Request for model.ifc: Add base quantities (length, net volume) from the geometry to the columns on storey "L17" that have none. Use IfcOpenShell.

First a look at what the model holds.

```python
import ifcopenshell
import ifcopenshell.util.element
import ifcopenshell.util.unit

model = ifcopenshell.open("model.ifc")
print(model.schema)
for unit_type in ("LENGTHUNIT", "AREAUNIT", "VOLUMEUNIT"):
    print(unit_type, ifcopenshell.util.unit.calculate_unit_scale(model, unit_type))
storey = next(s for s in model.by_type("IfcBuildingStorey") if s.Name == "L17")
columns = [e for e in ifcopenshell.util.element.get_decomposition(storey) if e.is_a("IfcColumn")]
for e in sorted(columns, key=lambda e: e.id()):
    print(e.id(), e.is_a(), e.Name, list(ifcopenshell.util.element.get_psets(e, qtos_only=True)), sep=" | ")
```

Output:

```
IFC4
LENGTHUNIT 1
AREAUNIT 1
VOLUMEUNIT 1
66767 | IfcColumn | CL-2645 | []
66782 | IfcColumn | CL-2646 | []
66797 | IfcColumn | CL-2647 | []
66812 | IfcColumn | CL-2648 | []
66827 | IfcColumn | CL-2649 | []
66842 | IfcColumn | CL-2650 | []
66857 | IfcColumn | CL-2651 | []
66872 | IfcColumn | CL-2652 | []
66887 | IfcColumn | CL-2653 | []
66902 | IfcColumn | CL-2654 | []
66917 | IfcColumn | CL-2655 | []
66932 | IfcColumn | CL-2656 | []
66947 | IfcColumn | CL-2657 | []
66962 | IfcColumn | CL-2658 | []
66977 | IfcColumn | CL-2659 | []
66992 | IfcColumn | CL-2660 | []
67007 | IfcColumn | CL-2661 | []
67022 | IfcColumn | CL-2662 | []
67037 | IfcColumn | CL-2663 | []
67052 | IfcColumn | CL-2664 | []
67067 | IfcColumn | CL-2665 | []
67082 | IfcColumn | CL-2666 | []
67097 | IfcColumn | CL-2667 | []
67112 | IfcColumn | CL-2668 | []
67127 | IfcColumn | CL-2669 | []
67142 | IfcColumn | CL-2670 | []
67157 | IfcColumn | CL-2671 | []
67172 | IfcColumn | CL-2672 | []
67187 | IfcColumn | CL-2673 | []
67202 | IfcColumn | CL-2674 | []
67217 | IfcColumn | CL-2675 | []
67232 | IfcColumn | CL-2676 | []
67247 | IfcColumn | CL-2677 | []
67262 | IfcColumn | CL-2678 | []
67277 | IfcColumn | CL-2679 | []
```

```python
import ifcopenshell
import ifcopenshell.api.pset
import ifcopenshell.geom
import ifcopenshell.util.element
import ifcopenshell.util.shape
import ifcopenshell.util.unit

model = ifcopenshell.open("model.ifc")
unit_scale = ifcopenshell.util.unit.calculate_unit_scale(model)
volume_scale = ifcopenshell.util.unit.calculate_unit_scale(model, "VOLUMEUNIT")
settings = ifcopenshell.geom.settings()

storey = next(s for s in model.by_type("IfcBuildingStorey") if s.Name == "L17")
columns = [e for e in ifcopenshell.util.element.get_decomposition(storey) if e.is_a("IfcColumn")]

for e in sorted(columns, key=lambda e: e.id()):
    if ifcopenshell.util.element.get_psets(e, qtos_only=True, should_inherit=False):
        continue
    # Geometry comes back in metres, in the element's own axes.
    shape = ifcopenshell.geom.create_shape(settings, e)
    values = {
        "Length": ifcopenshell.util.shape.get_z(shape.geometry) / unit_scale,
        "NetVolume": ifcopenshell.util.shape.get_volume(shape.geometry) / volume_scale,
    }
    qto = ifcopenshell.api.pset.add_qto(model, product=e, name="Qto_ColumnBaseQuantities")
    ifcopenshell.api.pset.edit_qto(model, qto=qto, properties=values)
    print(e.id(), {k: round(v, 3) for k, v in values.items()})

model.write("model_updated.ifc")
```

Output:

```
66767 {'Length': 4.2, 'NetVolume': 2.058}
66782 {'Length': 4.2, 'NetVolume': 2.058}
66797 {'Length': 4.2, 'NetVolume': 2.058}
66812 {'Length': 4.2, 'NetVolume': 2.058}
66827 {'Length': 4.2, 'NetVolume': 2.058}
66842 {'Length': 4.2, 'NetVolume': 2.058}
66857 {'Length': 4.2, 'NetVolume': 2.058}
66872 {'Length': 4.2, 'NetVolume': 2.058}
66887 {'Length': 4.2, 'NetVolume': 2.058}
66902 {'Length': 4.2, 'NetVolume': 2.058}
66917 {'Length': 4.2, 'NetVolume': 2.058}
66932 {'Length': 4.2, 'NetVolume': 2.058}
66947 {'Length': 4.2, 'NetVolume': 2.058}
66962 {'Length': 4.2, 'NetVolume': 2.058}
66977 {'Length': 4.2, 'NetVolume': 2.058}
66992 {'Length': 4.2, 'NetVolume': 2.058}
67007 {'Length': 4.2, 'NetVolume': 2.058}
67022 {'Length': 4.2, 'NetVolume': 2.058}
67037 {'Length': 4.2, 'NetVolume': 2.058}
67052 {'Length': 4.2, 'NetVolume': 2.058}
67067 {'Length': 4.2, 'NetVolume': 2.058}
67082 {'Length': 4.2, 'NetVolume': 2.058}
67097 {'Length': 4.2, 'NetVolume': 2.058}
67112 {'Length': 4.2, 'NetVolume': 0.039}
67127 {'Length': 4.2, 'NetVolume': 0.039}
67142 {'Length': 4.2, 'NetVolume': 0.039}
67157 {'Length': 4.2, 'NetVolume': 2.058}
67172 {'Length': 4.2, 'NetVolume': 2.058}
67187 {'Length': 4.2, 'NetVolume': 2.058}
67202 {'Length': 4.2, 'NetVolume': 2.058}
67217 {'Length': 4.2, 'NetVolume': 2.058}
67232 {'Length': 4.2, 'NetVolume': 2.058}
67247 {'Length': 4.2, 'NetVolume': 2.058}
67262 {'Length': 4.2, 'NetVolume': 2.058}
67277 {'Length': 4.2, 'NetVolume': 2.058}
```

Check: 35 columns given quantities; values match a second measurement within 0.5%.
